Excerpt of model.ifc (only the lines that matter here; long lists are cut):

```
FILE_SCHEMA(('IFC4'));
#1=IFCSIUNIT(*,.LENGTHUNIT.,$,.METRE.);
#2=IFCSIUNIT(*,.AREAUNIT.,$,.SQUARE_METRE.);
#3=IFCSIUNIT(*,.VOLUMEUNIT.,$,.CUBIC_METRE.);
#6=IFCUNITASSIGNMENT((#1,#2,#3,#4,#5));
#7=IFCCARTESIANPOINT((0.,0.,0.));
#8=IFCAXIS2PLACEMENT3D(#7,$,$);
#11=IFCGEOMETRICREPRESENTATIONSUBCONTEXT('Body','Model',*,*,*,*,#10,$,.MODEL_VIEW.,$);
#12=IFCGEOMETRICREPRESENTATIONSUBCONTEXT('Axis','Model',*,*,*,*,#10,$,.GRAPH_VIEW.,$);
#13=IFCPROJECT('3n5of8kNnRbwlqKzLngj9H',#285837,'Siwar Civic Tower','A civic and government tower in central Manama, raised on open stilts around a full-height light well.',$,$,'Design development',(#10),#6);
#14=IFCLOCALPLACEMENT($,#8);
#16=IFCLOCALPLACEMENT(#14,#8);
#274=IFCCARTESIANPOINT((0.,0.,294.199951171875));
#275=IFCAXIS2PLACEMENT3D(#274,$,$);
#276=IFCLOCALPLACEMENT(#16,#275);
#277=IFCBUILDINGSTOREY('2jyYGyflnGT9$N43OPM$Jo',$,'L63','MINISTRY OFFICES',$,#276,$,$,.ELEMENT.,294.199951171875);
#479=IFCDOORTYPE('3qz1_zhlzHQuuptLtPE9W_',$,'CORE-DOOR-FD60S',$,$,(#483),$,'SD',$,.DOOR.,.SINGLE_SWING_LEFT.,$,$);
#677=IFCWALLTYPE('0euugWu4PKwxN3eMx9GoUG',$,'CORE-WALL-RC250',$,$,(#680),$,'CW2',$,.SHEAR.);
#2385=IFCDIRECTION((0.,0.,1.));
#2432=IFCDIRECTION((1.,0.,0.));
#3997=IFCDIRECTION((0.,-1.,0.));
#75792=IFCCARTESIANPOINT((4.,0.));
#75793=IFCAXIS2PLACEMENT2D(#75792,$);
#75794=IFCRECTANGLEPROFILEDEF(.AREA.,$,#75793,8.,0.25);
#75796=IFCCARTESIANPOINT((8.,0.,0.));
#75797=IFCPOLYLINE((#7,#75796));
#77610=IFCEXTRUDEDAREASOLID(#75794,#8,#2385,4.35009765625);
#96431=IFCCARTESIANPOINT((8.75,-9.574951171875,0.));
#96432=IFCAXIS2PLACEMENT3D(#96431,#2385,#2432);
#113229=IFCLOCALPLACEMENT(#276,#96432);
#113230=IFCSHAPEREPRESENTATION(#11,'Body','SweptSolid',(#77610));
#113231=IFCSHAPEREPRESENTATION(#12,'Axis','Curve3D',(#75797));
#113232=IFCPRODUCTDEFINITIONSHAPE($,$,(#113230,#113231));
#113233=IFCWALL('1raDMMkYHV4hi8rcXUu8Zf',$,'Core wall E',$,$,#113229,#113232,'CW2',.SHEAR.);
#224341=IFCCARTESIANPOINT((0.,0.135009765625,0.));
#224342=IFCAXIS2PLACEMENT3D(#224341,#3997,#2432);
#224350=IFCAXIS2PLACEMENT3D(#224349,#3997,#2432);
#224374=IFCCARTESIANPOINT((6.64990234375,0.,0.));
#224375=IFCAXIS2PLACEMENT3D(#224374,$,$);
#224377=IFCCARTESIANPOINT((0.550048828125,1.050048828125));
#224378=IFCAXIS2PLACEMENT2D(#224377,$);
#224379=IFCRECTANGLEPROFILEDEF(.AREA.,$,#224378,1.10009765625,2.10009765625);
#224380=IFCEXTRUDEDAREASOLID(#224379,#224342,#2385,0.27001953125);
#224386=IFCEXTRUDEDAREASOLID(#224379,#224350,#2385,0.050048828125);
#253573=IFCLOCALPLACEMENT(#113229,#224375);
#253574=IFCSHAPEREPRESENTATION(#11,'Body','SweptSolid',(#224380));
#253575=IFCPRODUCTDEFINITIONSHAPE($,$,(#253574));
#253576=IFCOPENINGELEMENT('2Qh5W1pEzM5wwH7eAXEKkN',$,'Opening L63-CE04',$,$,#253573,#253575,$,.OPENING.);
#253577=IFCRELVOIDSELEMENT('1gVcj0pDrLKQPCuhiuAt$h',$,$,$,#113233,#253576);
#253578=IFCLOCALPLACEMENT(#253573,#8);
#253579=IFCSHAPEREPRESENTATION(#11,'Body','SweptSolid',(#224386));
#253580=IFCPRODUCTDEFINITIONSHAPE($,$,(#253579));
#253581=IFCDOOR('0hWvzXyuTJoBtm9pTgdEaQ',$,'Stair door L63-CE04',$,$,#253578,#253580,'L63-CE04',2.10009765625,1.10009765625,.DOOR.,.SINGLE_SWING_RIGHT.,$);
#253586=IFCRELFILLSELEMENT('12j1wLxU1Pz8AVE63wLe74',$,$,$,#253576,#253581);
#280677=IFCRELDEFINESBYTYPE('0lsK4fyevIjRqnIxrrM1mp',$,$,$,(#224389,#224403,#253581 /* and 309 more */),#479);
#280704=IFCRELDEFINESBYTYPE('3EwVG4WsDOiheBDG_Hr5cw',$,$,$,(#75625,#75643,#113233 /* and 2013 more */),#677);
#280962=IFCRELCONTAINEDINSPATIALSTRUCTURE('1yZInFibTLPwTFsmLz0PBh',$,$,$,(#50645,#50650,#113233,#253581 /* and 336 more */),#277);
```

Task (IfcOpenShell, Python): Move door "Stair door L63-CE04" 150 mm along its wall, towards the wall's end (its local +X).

```python
import ifcopenshell
import ifcopenshell.api.geometry
import ifcopenshell.util.placement
import ifcopenshell.util.unit

model = ifcopenshell.open("model.ifc")
unit_scale = ifcopenshell.util.unit.calculate_unit_scale(model)

door = model.by_guid("0hWvzXyuTJoBtm9pTgdEaQ")
opening = door.FillsVoids[0].RelatingOpeningElement
wall = opening.VoidsElements[0].RelatingBuildingElement

wall_matrix = ifcopenshell.util.placement.get_local_placement(wall.ObjectPlacement)
shift = wall_matrix[:3, 0] * 0.15 / unit_scale
before = ifcopenshell.util.placement.get_local_placement(door.ObjectPlacement)[:3, 3].copy()

# The door is placed relative to its opening, so it follows when the opening moves.
matrix = ifcopenshell.util.placement.get_local_placement(opening.ObjectPlacement)
matrix[:3, 3] += shift
ifcopenshell.api.geometry.edit_object_placement(
    model, product=opening, matrix=matrix, is_si=False, should_transform_children=True
)

after = ifcopenshell.util.placement.get_local_placement(door.ObjectPlacement)[:3, 3]
print("door moved by", (after - before).round(3) + 0.0)

model.write("model_updated.ifc")
```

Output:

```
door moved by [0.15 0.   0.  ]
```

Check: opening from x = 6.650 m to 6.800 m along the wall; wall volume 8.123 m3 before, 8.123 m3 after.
